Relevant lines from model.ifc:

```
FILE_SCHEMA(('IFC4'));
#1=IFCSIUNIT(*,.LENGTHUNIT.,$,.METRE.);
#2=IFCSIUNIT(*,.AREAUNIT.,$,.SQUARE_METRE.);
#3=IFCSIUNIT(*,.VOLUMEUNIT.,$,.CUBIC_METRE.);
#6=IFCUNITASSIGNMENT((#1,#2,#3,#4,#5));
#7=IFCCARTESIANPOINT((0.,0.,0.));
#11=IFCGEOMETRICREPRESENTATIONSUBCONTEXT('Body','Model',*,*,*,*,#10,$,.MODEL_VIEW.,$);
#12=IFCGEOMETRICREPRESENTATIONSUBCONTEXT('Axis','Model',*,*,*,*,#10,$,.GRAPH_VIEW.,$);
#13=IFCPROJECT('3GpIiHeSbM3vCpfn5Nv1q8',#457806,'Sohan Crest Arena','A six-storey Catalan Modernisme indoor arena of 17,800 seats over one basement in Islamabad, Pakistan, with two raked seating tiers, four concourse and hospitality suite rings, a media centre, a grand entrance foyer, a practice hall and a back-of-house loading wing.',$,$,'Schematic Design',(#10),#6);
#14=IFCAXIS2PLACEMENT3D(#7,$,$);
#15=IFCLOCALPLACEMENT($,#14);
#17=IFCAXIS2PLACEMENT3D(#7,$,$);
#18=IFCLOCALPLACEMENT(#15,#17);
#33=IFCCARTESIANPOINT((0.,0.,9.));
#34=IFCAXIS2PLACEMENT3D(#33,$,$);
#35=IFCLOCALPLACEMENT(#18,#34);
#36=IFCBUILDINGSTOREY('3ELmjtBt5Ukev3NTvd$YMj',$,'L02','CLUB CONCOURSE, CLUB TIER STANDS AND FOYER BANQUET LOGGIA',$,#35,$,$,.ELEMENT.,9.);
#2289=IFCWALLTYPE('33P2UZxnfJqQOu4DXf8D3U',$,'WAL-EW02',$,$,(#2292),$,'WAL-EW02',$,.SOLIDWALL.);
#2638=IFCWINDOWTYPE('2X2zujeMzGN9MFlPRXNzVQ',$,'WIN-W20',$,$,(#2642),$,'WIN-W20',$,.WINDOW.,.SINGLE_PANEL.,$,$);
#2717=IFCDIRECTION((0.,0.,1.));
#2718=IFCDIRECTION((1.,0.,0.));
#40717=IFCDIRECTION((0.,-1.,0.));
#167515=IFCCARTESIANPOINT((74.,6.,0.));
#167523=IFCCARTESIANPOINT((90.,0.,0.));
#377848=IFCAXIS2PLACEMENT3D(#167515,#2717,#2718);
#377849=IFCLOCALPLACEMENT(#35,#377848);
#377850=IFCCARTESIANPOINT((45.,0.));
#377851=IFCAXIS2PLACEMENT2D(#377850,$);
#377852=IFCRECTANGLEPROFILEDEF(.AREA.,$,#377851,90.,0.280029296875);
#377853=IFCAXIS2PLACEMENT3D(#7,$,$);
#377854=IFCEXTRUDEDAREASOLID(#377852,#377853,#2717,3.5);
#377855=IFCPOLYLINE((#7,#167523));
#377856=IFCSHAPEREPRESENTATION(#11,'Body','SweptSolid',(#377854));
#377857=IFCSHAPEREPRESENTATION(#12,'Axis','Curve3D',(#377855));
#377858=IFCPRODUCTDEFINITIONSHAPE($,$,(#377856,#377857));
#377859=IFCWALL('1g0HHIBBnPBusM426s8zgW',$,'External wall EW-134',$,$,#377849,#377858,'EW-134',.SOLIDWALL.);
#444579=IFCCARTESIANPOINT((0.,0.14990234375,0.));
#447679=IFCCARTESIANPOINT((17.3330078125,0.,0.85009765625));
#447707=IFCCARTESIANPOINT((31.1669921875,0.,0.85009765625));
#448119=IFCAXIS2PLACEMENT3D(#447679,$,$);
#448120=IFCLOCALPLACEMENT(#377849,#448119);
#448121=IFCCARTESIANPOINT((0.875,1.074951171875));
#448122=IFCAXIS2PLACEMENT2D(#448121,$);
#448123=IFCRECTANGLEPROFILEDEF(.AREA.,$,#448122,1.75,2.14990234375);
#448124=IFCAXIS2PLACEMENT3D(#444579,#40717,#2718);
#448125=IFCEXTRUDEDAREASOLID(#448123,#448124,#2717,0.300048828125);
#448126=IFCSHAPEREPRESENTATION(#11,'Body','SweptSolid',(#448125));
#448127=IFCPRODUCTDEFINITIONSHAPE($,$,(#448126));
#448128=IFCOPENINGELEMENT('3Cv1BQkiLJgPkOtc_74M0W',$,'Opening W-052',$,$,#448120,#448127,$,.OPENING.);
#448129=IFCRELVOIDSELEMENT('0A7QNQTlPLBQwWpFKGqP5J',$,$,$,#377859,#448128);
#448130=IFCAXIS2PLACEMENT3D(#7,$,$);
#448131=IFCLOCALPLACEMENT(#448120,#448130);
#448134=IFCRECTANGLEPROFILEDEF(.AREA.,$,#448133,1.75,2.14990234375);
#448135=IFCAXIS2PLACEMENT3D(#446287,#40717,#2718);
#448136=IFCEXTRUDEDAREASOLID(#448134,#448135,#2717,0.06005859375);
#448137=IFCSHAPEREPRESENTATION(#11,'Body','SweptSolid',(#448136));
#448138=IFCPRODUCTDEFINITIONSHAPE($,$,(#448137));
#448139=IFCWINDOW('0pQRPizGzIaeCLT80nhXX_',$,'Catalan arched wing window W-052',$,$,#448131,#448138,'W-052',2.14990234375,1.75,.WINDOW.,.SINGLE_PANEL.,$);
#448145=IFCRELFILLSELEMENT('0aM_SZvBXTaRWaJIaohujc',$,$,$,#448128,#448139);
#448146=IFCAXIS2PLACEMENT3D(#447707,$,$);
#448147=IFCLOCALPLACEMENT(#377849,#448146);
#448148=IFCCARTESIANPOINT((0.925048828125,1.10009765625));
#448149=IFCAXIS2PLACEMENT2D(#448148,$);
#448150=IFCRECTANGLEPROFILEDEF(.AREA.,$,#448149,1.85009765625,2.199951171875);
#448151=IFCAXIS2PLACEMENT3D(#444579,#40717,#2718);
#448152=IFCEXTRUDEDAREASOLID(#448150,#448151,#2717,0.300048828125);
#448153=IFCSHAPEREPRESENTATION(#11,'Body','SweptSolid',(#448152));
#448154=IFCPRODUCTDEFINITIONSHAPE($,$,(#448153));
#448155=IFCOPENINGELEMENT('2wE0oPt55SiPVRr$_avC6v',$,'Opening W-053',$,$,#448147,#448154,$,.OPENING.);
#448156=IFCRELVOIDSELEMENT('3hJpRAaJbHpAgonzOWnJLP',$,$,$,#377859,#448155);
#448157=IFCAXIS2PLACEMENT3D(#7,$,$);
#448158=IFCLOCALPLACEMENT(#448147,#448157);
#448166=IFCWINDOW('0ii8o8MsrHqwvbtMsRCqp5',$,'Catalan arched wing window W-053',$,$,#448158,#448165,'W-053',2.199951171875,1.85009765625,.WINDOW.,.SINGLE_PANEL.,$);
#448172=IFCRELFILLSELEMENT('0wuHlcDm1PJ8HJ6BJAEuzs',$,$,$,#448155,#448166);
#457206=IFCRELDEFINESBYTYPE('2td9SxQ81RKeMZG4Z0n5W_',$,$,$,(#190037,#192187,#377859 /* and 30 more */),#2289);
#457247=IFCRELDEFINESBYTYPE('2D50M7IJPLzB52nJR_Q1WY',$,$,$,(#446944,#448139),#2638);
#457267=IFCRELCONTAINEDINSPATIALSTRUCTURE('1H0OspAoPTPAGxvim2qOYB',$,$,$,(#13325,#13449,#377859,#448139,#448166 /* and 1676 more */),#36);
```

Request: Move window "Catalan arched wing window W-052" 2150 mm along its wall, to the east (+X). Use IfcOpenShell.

```python
import ifcopenshell
import ifcopenshell.api.geometry
import ifcopenshell.util.placement

model = ifcopenshell.open("model.ifc")

window = model.by_guid("0pQRPizGzIaeCLT80nhXX_")
opening = window.FillsVoids[0].RelatingOpeningElement
wall = opening.VoidsElements[0].RelatingBuildingElement

wall_matrix = ifcopenshell.util.placement.get_local_placement(wall.ObjectPlacement)
shift = wall_matrix[:3, 0] * 2.15
before = ifcopenshell.util.placement.get_local_placement(window.ObjectPlacement)[:3, 3].copy()

# The window is placed relative to its opening, so it follows when the opening moves.
matrix = ifcopenshell.util.placement.get_local_placement(opening.ObjectPlacement)
matrix[:3, 3] += shift
ifcopenshell.api.geometry.edit_object_placement(
    model, product=opening, matrix=matrix, is_si=False, should_transform_children=True
)

after = ifcopenshell.util.placement.get_local_placement(window.ObjectPlacement)[:3, 3]
print("window moved by", (after - before).round(3) + 0.0)

model.write("model_rev.ifc")
```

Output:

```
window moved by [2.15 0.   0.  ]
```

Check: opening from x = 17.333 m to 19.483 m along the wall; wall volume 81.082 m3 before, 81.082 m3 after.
